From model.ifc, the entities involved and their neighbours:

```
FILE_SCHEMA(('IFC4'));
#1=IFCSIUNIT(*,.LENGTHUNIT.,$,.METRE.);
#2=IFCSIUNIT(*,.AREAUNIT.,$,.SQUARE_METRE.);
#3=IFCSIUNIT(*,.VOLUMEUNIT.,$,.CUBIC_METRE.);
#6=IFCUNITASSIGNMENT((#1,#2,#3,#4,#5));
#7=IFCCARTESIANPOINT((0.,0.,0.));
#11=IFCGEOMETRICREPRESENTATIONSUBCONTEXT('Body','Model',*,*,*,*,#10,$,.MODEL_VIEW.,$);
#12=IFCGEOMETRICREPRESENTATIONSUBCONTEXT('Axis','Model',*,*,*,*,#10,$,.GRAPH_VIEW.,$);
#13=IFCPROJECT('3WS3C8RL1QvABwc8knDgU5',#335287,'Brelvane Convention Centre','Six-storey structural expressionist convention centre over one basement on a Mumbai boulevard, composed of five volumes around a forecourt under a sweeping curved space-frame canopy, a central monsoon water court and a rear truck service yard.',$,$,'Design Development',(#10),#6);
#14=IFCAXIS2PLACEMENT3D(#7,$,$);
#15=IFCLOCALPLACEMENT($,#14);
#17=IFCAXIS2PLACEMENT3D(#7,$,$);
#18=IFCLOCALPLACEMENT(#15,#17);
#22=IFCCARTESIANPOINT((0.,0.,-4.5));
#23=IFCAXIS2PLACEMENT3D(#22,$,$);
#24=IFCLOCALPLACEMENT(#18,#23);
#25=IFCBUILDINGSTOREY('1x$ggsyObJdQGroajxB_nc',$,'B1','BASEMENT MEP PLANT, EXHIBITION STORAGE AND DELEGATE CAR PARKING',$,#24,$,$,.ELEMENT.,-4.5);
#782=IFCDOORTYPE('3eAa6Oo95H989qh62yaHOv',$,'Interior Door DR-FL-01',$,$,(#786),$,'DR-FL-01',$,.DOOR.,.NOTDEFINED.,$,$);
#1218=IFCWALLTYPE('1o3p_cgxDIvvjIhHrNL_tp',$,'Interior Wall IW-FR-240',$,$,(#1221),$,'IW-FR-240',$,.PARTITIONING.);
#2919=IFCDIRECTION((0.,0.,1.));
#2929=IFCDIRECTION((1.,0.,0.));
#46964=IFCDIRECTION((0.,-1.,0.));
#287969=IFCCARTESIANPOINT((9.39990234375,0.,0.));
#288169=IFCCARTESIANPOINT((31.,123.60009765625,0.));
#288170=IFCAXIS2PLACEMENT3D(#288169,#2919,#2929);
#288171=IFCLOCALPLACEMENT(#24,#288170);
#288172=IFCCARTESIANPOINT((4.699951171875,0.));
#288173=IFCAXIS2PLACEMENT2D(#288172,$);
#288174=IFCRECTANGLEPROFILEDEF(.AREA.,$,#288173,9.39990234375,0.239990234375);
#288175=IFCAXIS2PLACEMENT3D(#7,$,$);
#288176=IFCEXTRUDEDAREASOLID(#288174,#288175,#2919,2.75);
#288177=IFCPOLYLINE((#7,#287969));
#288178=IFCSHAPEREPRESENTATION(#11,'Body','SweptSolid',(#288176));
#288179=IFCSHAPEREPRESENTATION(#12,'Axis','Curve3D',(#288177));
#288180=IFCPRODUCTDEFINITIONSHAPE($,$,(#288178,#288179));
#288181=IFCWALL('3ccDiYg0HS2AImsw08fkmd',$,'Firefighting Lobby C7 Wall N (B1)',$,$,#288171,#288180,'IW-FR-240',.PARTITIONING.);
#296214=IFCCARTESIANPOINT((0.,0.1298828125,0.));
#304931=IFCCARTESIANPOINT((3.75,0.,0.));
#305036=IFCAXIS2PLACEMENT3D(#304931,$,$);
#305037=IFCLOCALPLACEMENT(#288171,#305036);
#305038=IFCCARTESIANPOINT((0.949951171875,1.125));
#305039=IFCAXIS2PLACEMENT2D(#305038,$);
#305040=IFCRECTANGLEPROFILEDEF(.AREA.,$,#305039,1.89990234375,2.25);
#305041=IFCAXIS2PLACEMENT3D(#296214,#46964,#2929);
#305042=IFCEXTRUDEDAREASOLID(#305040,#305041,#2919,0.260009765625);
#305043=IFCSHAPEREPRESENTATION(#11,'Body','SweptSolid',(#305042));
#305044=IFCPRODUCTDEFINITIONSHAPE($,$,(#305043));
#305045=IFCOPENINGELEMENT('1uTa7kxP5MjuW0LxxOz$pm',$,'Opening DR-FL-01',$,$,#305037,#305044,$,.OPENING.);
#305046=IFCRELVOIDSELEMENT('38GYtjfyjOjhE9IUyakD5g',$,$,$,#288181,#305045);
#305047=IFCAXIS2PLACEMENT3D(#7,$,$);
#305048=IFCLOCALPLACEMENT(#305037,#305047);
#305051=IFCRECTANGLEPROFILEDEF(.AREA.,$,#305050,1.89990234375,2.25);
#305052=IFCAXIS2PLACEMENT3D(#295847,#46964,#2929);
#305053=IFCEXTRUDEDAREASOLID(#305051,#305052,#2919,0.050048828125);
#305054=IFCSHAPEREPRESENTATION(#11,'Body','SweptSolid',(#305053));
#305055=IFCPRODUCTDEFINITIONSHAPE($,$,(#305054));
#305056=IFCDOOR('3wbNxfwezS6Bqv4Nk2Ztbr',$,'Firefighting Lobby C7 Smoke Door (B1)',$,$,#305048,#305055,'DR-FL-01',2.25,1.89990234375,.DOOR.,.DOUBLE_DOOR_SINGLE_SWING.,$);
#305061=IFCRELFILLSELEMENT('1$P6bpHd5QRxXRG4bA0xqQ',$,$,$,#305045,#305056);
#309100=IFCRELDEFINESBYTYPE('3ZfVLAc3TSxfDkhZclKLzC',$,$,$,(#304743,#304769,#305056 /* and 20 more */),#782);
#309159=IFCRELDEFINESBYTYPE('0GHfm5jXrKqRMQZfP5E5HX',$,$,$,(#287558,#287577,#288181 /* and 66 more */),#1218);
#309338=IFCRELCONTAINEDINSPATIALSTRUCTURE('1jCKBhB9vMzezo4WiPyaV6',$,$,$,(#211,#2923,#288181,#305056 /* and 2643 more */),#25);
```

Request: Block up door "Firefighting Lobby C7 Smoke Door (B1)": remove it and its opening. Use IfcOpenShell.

```python
import ifcopenshell
import ifcopenshell.api.feature
import ifcopenshell.api.root
import ifcopenshell.geom
import ifcopenshell.util.shape

model = ifcopenshell.open("model.ifc")
settings = ifcopenshell.geom.settings()


def volume(element):
    """Net volume in cubic metres, openings subtracted."""
    shape = ifcopenshell.geom.create_shape(settings, element)
    return ifcopenshell.util.shape.get_volume(shape.geometry)


door = model.by_guid("3wbNxfwezS6Bqv4Nk2Ztbr")
opening = door.FillsVoids[0].RelatingOpeningElement
wall = opening.VoidsElements[0].RelatingBuildingElement
before = volume(wall)

ifcopenshell.api.root.remove_product(model, product=door)
ifcopenshell.api.feature.remove_feature(model, feature=opening)

after = volume(wall)

print(f"wall volume {before:.3f} -> {after:.3f} m3")

model.write("model_updated.ifc")
```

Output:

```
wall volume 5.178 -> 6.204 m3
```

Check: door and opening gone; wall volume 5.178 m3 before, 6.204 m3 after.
